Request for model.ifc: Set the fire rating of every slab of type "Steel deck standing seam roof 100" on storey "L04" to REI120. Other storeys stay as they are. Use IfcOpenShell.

First a look at what the model holds.

```python
import ifcopenshell
import ifcopenshell.util.element

model = ifcopenshell.open("model.ifc")
print(model.schema)
storey = next(s for s in model.by_type("IfcBuildingStorey") if s.Name == "L04")
slabs = [e for e in ifcopenshell.util.element.get_decomposition(storey) if e.is_a("IfcSlab")]
seen = {}
for e in slabs:
    element_type = ifcopenshell.util.element.get_type(e)
    key = (element_type.Name if element_type != e and element_type else None, ifcopenshell.util.element.get_pset(e, "Pset_SlabCommon", "FireRating"))
    seen[key] = seen.get(key, 0) + 1
for (name, value), count in sorted(seen.items(), key=str):
    print(count, "x", name, "|", value)
```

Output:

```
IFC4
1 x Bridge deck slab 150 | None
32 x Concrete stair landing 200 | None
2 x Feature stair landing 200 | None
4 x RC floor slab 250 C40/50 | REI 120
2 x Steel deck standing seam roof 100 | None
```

```python
import ifcopenshell
import ifcopenshell.api.pset
import ifcopenshell.util.element

model = ifcopenshell.open("model.ifc")

storey = next(s for s in model.by_type("IfcBuildingStorey") if s.Name == "L04")
slabs = [e for e in ifcopenshell.util.element.get_decomposition(storey) if e.is_a("IfcSlab")]

count = 0
for e in slabs:
    element_type = ifcopenshell.util.element.get_type(e)
    if element_type in (None, e) or element_type.Name != "Steel deck standing seam roof 100":
        continue
    # add_pset returns the element's existing set when there is one.
    pset = ifcopenshell.api.pset.add_pset(model, product=e, name="Pset_SlabCommon")
    ifcopenshell.api.pset.edit_pset(model, pset=pset, properties={"FireRating": "REI120"})
    count += 1

print(count, "slabs updated")

model.write("model_updated.ifc")
```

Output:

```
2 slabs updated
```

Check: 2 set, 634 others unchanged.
